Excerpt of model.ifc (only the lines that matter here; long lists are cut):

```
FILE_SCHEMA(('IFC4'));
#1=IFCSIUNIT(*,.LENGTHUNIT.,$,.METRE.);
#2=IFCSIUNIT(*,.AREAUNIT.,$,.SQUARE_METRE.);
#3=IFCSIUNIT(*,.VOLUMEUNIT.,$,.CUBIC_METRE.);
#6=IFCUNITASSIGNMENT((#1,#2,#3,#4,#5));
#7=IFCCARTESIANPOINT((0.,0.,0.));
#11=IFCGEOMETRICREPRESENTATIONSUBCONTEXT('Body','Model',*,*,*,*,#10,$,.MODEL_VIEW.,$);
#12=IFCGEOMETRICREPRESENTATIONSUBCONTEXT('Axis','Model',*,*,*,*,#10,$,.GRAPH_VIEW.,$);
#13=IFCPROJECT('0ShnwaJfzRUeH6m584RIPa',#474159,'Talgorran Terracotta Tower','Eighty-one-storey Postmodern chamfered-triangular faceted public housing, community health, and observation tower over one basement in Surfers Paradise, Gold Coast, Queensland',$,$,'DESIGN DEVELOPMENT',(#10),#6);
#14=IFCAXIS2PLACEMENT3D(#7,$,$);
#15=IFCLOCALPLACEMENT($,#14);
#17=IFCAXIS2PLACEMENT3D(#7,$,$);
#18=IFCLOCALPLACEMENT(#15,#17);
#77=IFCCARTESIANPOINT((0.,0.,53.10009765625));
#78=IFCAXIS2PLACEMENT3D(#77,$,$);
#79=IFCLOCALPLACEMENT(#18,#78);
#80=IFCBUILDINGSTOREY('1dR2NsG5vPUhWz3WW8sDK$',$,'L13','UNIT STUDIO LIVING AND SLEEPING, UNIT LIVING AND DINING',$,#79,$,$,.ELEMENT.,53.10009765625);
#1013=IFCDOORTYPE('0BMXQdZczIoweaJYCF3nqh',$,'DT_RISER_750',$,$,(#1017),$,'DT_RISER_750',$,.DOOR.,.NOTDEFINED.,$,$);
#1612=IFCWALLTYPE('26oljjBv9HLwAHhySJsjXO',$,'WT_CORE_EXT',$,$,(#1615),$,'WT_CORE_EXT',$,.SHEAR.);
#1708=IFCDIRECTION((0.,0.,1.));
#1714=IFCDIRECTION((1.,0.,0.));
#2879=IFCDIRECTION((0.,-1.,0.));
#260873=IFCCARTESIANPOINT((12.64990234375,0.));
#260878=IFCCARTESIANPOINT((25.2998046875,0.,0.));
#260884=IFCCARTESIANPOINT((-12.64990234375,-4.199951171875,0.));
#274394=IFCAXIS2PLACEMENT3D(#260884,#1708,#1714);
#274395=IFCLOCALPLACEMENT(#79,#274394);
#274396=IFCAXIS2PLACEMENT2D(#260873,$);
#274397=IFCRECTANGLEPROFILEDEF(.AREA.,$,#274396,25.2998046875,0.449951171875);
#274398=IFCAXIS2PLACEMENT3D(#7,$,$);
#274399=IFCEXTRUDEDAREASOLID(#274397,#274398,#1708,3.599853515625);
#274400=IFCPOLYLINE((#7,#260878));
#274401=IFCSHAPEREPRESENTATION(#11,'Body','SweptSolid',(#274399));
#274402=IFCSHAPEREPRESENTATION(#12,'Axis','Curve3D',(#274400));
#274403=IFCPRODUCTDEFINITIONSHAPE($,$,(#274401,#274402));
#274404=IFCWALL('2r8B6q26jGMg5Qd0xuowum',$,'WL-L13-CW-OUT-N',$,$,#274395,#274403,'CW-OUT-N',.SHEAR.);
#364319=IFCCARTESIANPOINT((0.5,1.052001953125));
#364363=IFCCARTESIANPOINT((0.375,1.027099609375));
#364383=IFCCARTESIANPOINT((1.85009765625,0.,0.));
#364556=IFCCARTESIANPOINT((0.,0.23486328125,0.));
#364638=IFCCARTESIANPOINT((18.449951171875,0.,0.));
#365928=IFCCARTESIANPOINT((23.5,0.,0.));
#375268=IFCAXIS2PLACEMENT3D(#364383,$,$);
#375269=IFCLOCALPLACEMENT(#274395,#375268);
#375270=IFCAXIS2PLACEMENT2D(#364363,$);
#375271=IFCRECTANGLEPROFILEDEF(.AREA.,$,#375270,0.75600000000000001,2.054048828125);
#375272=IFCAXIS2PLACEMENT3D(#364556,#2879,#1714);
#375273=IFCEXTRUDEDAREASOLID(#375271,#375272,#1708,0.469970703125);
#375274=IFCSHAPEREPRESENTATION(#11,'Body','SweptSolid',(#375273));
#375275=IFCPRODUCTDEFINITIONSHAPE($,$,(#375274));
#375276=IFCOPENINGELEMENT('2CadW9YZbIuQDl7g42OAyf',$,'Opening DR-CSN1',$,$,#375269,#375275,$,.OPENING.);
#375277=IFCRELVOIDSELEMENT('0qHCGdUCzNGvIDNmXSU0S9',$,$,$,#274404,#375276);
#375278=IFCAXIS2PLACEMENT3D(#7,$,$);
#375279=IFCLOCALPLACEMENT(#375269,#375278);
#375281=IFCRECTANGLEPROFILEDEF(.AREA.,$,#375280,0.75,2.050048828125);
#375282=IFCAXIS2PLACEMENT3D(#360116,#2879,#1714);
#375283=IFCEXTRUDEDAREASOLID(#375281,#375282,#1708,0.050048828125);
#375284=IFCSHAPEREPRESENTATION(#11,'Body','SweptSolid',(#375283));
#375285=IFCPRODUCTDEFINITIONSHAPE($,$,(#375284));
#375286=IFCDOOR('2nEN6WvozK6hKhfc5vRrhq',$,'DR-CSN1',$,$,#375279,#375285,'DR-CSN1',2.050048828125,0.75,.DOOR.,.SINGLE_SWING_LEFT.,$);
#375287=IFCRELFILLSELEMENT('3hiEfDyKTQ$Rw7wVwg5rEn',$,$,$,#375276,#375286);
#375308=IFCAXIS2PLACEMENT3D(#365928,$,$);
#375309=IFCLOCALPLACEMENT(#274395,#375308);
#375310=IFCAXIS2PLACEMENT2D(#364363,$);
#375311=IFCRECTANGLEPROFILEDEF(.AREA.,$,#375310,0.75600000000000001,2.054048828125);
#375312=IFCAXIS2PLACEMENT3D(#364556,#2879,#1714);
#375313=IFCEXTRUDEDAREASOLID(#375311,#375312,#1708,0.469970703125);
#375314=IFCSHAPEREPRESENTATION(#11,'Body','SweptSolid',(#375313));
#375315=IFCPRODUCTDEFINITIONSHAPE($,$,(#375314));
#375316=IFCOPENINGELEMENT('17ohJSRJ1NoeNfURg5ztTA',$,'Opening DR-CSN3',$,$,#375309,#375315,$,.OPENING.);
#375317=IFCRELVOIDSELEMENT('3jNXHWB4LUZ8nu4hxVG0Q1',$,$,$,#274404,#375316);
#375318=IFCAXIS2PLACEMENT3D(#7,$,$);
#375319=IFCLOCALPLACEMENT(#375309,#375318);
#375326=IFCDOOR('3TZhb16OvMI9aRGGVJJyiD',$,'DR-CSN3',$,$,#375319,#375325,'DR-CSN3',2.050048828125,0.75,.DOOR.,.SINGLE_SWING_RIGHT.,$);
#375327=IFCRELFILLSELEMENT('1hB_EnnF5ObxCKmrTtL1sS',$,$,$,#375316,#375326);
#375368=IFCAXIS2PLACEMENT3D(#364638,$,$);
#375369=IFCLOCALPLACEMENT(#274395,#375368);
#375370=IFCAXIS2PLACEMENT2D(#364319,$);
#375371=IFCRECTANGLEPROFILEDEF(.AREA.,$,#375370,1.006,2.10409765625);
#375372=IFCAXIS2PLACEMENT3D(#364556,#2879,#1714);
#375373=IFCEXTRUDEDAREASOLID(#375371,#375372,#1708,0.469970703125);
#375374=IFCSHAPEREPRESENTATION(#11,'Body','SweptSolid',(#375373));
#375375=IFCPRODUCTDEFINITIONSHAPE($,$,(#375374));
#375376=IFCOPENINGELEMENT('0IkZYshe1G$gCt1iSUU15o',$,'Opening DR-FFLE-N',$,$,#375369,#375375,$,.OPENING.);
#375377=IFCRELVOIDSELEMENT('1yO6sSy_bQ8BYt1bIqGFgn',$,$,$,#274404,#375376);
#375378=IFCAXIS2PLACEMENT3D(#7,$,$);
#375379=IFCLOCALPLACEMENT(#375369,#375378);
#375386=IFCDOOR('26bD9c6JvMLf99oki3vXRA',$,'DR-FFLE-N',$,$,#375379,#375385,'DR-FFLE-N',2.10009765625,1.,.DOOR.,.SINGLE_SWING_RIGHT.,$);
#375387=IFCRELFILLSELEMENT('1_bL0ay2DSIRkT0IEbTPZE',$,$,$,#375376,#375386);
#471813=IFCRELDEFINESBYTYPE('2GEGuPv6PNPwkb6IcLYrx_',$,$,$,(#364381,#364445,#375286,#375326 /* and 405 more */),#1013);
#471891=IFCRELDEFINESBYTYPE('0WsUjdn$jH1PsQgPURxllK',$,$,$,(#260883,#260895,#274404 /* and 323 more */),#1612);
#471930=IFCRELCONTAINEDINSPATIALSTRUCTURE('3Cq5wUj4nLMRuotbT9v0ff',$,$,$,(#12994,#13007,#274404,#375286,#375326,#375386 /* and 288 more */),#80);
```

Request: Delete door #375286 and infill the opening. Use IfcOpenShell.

```python
import ifcopenshell
import ifcopenshell.api.feature
import ifcopenshell.api.root
import ifcopenshell.geom
import ifcopenshell.util.shape

model = ifcopenshell.open("model.ifc")
settings = ifcopenshell.geom.settings()


def volume(element):
    """Net volume in cubic metres, openings subtracted."""
    shape = ifcopenshell.geom.create_shape(settings, element)
    return ifcopenshell.util.shape.get_volume(shape.geometry)


door = model.by_guid("2nEN6WvozK6hKhfc5vRrhq")
opening = door.FillsVoids[0].RelatingOpeningElement
wall = opening.VoidsElements[0].RelatingBuildingElement
before = volume(wall)

ifcopenshell.api.root.remove_product(model, product=door)
ifcopenshell.api.feature.remove_feature(model, feature=opening)

after = volume(wall)

print(f"wall volume {before:.3f} -> {after:.3f} m3")

model.write("model_edited.ifc")
```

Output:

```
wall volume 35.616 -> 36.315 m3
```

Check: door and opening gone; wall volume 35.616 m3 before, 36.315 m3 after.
